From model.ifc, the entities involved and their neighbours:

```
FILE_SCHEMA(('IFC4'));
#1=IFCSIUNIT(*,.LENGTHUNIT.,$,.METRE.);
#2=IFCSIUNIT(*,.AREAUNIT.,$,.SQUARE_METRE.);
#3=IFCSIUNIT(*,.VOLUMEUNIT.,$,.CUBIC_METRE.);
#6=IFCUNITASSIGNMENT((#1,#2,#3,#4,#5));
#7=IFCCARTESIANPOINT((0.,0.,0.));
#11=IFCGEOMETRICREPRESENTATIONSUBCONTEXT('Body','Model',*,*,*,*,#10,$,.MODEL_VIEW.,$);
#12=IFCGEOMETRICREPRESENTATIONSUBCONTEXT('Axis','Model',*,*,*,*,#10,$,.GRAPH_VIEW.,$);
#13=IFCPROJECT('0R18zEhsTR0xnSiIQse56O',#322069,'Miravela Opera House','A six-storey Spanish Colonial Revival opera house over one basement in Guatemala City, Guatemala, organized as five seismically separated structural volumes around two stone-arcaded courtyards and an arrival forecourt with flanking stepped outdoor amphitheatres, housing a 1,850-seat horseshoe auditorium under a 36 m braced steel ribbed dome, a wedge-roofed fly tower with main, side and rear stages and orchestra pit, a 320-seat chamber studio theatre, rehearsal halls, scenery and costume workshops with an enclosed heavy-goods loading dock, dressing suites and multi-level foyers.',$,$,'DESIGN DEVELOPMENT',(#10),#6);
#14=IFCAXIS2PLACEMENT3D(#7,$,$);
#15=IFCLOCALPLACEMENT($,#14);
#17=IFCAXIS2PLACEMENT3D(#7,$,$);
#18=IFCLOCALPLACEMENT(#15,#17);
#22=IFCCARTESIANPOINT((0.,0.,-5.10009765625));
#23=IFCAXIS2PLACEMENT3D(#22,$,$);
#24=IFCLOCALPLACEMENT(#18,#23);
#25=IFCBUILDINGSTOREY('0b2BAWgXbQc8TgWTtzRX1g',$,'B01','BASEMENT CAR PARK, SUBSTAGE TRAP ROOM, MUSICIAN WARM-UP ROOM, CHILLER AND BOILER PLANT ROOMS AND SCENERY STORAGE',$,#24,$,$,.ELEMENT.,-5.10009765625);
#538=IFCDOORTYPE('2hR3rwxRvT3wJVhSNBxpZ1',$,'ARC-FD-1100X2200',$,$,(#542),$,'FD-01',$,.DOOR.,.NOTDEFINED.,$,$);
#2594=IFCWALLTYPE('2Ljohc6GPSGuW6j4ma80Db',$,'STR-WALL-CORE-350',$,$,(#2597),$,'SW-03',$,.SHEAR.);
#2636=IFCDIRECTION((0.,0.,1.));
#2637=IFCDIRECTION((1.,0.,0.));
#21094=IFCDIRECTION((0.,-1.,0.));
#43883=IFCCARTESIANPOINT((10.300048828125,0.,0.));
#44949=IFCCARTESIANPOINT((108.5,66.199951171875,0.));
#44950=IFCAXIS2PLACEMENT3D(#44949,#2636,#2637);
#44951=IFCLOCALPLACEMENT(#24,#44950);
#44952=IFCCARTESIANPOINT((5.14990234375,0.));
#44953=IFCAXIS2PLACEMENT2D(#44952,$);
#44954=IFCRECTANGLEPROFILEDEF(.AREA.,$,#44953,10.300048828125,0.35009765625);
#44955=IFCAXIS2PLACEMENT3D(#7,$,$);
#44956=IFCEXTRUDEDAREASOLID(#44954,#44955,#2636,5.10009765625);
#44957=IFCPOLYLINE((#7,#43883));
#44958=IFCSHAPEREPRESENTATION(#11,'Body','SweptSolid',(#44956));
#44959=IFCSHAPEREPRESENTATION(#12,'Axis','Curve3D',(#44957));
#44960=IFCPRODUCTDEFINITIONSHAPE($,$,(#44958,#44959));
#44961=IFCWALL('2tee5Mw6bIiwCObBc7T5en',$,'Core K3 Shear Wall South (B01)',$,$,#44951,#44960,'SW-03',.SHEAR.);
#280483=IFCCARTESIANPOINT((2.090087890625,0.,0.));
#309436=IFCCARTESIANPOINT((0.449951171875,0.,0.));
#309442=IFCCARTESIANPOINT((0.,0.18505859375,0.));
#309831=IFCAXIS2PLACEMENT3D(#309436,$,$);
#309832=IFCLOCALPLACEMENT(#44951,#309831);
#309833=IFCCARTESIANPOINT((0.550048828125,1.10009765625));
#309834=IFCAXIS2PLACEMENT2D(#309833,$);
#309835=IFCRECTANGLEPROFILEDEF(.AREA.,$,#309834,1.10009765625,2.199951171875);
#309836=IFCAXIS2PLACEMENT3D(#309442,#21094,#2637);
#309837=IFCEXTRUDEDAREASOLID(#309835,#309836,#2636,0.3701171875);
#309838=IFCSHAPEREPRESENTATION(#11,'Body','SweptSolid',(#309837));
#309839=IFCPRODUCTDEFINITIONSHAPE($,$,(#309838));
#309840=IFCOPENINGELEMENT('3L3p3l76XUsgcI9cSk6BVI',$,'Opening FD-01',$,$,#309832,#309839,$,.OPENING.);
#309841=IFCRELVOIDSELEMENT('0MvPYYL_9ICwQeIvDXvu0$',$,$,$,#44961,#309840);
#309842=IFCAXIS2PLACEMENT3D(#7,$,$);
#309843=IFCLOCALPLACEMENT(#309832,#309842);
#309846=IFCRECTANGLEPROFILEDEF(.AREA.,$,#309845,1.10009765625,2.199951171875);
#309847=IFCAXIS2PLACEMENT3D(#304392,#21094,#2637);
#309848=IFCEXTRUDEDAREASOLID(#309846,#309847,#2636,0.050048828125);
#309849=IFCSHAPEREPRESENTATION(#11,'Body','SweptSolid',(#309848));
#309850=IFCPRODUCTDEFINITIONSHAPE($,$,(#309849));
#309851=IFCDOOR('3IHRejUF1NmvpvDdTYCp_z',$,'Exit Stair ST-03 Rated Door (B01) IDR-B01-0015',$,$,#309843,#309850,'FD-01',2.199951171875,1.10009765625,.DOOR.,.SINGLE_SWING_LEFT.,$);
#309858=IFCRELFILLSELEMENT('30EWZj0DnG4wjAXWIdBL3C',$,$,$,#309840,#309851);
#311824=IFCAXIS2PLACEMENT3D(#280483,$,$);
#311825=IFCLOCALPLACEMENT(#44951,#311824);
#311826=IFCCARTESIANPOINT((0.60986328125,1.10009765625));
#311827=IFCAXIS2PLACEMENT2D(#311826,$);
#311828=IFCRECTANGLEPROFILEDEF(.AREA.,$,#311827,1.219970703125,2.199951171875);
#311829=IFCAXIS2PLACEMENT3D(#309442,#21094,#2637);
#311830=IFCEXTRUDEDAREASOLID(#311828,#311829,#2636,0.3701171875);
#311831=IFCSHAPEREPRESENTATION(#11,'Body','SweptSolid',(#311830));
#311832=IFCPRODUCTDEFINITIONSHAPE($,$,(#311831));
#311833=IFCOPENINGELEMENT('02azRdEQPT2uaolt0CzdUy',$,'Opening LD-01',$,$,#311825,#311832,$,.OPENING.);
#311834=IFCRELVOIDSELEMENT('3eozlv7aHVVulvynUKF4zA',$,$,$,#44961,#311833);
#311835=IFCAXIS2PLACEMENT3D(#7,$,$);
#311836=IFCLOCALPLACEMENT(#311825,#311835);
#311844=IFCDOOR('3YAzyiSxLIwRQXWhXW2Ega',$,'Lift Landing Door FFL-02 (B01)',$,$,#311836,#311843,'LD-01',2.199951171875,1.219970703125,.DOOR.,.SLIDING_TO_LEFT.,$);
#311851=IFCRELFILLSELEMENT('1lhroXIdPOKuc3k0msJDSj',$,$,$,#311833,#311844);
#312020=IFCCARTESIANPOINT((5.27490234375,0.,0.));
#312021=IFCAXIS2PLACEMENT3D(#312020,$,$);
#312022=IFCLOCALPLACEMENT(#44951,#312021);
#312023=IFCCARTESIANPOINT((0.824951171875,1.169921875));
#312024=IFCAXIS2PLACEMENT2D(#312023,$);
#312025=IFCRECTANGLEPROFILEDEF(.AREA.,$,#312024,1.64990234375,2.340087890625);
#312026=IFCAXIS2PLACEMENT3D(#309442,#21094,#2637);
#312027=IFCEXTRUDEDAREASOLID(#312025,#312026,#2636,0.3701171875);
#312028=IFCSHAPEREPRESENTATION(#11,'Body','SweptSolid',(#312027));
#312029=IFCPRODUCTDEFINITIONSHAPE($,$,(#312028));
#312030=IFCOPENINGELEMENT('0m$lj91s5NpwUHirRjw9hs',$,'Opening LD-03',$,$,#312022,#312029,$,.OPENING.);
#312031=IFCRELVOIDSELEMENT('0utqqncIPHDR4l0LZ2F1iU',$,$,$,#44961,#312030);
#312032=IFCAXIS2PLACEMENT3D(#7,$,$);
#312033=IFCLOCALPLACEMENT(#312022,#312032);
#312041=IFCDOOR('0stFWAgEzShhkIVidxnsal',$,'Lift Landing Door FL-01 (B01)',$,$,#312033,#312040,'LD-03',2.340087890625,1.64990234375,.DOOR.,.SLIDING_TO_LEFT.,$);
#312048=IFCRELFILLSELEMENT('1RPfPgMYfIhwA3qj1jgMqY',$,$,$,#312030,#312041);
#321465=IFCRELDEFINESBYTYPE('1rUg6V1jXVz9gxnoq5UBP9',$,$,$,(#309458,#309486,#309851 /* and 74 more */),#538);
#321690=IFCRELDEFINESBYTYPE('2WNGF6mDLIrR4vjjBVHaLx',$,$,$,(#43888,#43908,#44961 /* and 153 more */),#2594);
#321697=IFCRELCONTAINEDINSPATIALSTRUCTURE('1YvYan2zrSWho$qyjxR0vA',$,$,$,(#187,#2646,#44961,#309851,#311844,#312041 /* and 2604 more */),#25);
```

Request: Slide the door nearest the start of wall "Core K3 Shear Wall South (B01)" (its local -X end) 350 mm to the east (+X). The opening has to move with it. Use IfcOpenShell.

```python
import ifcopenshell
import ifcopenshell.api.geometry
import ifcopenshell.util.placement
import ifcopenshell.util.unit

model = ifcopenshell.open("model.ifc")
unit_scale = ifcopenshell.util.unit.calculate_unit_scale(model)

door = model.by_guid("3IHRejUF1NmvpvDdTYCp_z")
opening = door.FillsVoids[0].RelatingOpeningElement
wall = opening.VoidsElements[0].RelatingBuildingElement

wall_matrix = ifcopenshell.util.placement.get_local_placement(wall.ObjectPlacement)
shift = wall_matrix[:3, 0] * 0.35 / unit_scale
before = ifcopenshell.util.placement.get_local_placement(door.ObjectPlacement)[:3, 3].copy()

# The door is placed relative to its opening, so it follows when the opening moves.
matrix = ifcopenshell.util.placement.get_local_placement(opening.ObjectPlacement)
matrix[:3, 3] += shift
ifcopenshell.api.geometry.edit_object_placement(
    model, product=opening, matrix=matrix, is_si=False, should_transform_children=True
)

after = ifcopenshell.util.placement.get_local_placement(door.ObjectPlacement)[:3, 3]
print("door moved by", (after - before).round(3) + 0.0)

model.write("model-out.ifc")
```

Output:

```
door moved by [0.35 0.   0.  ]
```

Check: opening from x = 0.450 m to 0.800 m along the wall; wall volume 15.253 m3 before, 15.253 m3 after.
